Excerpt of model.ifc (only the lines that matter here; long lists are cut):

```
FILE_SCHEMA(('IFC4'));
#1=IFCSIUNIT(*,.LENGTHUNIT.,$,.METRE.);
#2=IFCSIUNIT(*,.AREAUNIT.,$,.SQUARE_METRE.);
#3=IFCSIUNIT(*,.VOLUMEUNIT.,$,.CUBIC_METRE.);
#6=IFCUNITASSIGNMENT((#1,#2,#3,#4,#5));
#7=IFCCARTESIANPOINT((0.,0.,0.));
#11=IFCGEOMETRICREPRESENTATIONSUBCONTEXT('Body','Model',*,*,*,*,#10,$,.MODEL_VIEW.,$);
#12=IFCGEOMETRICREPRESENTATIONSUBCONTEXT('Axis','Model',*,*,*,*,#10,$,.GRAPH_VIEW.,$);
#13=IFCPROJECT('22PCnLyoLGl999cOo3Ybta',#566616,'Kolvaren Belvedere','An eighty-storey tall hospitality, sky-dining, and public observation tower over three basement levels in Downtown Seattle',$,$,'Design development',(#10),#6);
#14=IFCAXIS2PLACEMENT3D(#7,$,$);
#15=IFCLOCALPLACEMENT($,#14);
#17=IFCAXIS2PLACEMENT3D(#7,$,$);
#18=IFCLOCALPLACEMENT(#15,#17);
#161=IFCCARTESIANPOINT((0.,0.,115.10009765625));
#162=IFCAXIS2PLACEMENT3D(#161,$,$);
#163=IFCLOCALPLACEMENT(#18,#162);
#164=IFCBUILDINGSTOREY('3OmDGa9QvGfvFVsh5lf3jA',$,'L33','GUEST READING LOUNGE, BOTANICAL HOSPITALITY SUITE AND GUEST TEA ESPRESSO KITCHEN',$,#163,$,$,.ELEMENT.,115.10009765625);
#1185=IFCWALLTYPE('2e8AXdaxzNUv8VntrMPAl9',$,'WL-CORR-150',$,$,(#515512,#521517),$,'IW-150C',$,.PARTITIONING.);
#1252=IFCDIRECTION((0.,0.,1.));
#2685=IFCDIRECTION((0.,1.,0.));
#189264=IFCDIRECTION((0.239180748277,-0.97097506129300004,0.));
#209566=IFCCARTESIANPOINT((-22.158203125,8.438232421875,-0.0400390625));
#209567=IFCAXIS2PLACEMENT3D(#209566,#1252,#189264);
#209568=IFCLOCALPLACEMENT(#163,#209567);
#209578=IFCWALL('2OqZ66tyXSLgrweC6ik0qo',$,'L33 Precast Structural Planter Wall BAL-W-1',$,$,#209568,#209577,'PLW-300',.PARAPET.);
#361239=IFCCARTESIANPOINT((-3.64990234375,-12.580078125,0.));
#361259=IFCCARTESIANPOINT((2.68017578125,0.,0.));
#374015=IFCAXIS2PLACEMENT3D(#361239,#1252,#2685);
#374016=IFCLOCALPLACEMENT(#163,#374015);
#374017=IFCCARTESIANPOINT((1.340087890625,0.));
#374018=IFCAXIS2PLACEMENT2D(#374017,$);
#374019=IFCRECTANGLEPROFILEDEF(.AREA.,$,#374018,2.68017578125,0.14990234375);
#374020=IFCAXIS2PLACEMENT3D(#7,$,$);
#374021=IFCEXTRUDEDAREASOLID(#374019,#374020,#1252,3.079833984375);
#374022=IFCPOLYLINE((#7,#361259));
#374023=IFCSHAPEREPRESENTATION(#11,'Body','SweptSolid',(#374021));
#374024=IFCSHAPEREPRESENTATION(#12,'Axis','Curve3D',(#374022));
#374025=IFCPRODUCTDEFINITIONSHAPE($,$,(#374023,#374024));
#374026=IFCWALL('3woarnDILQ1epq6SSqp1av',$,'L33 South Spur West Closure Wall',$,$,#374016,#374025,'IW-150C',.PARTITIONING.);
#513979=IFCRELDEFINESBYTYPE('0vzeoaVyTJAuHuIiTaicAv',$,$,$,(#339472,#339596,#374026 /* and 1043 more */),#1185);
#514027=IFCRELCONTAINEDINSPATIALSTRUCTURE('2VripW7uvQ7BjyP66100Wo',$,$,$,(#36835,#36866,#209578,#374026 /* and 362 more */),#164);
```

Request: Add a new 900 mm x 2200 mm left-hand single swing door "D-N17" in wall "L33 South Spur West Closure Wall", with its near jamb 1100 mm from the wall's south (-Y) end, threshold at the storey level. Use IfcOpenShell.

```python
import numpy as np
import ifcopenshell
import ifcopenshell.api.feature
import ifcopenshell.api.geometry
import ifcopenshell.api.root
import ifcopenshell.api.spatial
import ifcopenshell.geom
import ifcopenshell.util.element
import ifcopenshell.util.placement
import ifcopenshell.util.representation
import ifcopenshell.util.shape
import ifcopenshell.util.unit

model = ifcopenshell.open("model.ifc")
unit_scale = ifcopenshell.util.unit.calculate_unit_scale(model)
settings = ifcopenshell.geom.settings()


def volume(element):
    """Net volume in cubic metres, openings subtracted."""
    shape = ifcopenshell.geom.create_shape(settings, element)
    return ifcopenshell.util.shape.get_volume(shape.geometry)


wall = model.by_id(374026)
storey = ifcopenshell.util.element.get_container(wall, ifc_class="IfcBuildingStorey")
context = ifcopenshell.util.representation.get_context(model, "Model", "Body", "MODEL_VIEW")
before = volume(wall)

width, height, from_end, sill = 0.9, 2.2, 1.1, 0.0  # metres

# The wall runs along its own X axis, and the end named is its -X end.
wall_shape = ifcopenshell.geom.create_shape(settings, wall)
x, y, z = ifcopenshell.util.shape.get_vertices(wall_shape.geometry).T
start = x.min() + from_end
face, thickness = float(y.min()), float(y.max() - y.min())
wall_matrix = ifcopenshell.util.placement.get_local_placement(wall.ObjectPlacement)
level = ifcopenshell.util.placement.get_local_placement(storey.ObjectPlacement)[2, 3]


def in_wall(x, y):
    """Placement at x, y metres in the wall's axes, at sill height."""
    matrix = wall_matrix.copy()
    matrix[:, 3] = wall_matrix @ np.array([x / unit_scale, y / unit_scale, 0.0, 1.0])
    matrix[2, 3] = level + sill / unit_scale
    return matrix


# Opening: a box that overshoots both wall faces by 50 mm.
opening = ifcopenshell.api.root.create_entity(model, ifc_class="IfcOpeningElement", predefined_type="OPENING")
box = ifcopenshell.api.geometry.add_wall_representation(
    model, context=context, length=width, height=height, thickness=thickness + 0.1
)
ifcopenshell.api.geometry.assign_representation(model, product=opening, representation=box)
ifcopenshell.api.geometry.edit_object_placement(model, product=opening, matrix=in_wall(start, face - 0.05), is_si=False)
ifcopenshell.api.feature.add_feature(model, feature=opening, element=wall)

door = ifcopenshell.api.root.create_entity(model, ifc_class="IfcDoor", name="D-N17", predefined_type="DOOR")
door.OverallWidth, door.OverallHeight = width / unit_scale, height / unit_scale
door.OperationType = "SINGLE_SWING_LEFT"
body = ifcopenshell.api.geometry.add_door_representation(
    model,
    context=context,
    overall_width=door.OverallWidth,
    overall_height=door.OverallHeight,
    operation_type="SINGLE_SWING_LEFT",
    lining_properties={"LiningDepth": thickness / unit_scale, "ThresholdDepth": thickness / unit_scale},
)
ifcopenshell.api.geometry.assign_representation(model, product=door, representation=body)
ifcopenshell.api.spatial.assign_container(model, products=[door], relating_structure=storey)
ifcopenshell.api.feature.add_filling(model, opening=opening, element=door)

# The lining spans the wall, so the door starts at the wall face.
ifcopenshell.api.geometry.edit_object_placement(model, product=door, matrix=in_wall(start, face), is_si=False)

after = volume(wall)

print(f"wall volume {before:.3f} -> {after:.3f} m3")

model.write("model_rev.ifc")
```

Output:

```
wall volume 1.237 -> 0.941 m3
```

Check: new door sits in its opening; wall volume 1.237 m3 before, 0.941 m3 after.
